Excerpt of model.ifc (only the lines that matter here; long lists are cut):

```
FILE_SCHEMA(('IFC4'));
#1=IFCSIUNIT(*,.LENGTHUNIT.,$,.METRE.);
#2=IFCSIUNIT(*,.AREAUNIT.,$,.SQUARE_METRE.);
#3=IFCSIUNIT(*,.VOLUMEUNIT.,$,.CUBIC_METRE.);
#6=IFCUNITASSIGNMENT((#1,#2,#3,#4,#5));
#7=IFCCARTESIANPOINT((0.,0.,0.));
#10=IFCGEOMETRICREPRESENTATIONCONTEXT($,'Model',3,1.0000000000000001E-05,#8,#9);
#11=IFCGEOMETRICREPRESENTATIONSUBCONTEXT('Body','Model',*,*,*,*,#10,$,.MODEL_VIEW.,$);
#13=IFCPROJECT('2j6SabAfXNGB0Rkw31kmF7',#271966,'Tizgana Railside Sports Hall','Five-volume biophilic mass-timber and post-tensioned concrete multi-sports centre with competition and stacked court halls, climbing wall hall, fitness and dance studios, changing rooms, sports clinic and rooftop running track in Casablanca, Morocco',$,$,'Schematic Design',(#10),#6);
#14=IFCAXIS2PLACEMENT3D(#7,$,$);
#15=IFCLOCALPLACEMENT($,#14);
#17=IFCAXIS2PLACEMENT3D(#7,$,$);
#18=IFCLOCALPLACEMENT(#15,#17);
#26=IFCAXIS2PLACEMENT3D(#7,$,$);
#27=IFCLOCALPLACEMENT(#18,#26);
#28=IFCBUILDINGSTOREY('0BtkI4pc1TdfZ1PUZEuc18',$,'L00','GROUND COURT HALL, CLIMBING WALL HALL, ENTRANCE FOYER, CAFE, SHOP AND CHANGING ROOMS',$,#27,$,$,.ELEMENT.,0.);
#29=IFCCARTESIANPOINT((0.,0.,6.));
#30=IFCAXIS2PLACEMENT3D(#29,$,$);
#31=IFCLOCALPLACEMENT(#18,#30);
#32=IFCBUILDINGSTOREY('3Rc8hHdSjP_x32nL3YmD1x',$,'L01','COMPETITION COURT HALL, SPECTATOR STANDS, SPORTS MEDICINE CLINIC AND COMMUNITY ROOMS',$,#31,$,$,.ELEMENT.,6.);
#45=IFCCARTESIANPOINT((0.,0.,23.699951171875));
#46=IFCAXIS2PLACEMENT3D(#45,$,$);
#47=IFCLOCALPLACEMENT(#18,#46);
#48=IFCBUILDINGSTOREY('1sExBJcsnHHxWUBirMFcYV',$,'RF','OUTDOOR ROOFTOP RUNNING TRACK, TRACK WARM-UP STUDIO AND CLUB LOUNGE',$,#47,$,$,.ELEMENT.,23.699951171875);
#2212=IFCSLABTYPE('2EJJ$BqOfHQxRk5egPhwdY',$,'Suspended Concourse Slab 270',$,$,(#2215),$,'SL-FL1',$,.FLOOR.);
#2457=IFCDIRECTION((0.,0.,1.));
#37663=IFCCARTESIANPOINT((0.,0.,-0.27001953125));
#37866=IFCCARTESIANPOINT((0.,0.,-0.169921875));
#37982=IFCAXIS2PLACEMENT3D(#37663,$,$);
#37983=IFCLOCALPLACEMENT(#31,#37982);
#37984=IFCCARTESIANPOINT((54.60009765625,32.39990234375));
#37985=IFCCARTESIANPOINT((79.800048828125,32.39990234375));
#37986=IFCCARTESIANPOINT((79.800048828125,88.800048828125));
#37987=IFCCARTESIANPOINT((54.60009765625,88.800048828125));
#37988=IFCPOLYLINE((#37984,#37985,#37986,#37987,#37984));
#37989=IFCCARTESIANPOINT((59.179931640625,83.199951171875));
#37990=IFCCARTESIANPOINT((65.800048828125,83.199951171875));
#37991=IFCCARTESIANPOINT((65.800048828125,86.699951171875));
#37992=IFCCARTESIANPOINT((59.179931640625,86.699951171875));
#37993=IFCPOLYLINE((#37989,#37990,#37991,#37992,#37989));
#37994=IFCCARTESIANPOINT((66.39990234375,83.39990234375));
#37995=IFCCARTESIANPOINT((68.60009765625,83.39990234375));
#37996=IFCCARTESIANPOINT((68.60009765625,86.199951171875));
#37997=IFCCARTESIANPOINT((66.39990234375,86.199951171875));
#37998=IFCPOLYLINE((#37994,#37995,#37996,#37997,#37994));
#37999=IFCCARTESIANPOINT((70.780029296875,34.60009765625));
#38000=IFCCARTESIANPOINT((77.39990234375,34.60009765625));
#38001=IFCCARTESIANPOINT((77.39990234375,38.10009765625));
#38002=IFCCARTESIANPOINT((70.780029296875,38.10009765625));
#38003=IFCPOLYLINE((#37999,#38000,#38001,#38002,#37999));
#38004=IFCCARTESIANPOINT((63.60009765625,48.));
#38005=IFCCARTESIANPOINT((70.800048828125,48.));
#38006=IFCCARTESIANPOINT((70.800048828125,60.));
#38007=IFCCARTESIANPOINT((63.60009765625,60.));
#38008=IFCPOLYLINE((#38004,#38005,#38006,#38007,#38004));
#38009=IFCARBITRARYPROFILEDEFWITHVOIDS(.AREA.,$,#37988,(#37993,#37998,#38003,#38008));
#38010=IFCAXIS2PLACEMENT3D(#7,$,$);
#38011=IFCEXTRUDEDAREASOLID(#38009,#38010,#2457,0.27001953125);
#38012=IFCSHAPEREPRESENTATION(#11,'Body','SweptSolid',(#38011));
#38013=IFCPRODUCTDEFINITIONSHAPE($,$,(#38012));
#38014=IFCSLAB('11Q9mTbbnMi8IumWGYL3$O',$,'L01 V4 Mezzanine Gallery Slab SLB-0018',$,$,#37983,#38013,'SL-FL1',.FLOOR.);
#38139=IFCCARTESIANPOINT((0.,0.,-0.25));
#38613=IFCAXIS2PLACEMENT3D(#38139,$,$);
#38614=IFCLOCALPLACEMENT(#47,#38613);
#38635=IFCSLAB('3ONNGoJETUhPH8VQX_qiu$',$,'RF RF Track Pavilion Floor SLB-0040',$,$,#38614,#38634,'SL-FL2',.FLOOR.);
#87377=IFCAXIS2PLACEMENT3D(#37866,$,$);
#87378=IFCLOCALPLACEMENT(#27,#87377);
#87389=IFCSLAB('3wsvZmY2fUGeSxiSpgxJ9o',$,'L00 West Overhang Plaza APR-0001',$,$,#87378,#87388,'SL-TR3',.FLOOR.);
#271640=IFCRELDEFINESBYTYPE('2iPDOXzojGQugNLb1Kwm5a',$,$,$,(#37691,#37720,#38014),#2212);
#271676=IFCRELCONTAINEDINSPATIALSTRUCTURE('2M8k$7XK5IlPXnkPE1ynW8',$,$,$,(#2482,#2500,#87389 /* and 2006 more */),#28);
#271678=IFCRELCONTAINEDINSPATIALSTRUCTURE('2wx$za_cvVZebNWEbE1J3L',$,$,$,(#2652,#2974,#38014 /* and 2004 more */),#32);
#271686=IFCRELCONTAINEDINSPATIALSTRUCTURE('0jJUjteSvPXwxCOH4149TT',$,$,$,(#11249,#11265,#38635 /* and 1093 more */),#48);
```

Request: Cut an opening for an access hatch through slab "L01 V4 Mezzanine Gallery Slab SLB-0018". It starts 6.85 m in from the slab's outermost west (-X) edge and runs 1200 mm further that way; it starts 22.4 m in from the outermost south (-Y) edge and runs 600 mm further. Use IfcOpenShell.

```python
import numpy as np
import ifcopenshell
import ifcopenshell.api.feature
import ifcopenshell.api.geometry
import ifcopenshell.api.root
import ifcopenshell.geom
import ifcopenshell.util.placement
import ifcopenshell.util.representation
import ifcopenshell.util.shape
import ifcopenshell.util.unit

model = ifcopenshell.open("model.ifc")
unit_scale = ifcopenshell.util.unit.calculate_unit_scale(model)
settings = ifcopenshell.geom.settings()


def volume(element):
    """Net volume in cubic metres, openings subtracted."""
    shape = ifcopenshell.geom.create_shape(settings, element)
    return ifcopenshell.util.shape.get_volume(shape.geometry)


slab = model.by_id(38014)
before = volume(slab)

# Extent in the slab's own axes, in metres. The edges named are its -X and -Y sides.
slab_shape = ifcopenshell.geom.create_shape(settings, slab)
vertices = ifcopenshell.util.shape.get_vertices(slab_shape.geometry)
x_min, y_min, bottom = vertices.min(axis=0)
top = vertices[:, 2].max()

opening = ifcopenshell.api.root.create_entity(model, ifc_class="IfcOpeningElement", name="Access hatch opening", predefined_type="OPENING")
context = ifcopenshell.util.representation.get_context(model, "Model", "Body", "MODEL_VIEW")
width, depth = 1.2, 0.6
outline = [(0.0, 0.0), (width, 0.0), (width, depth), (0.0, depth), (0.0, 0.0)]
# Overshoot both faces by 50 mm so the cut is clean.
shape = ifcopenshell.api.geometry.add_slab_representation(
    model, context=context, depth=top - bottom + 0.1, polyline=outline
)
ifcopenshell.api.geometry.assign_representation(model, product=opening, representation=shape)

matrix = ifcopenshell.util.placement.get_local_placement(slab.ObjectPlacement)
matrix[:, 3] = matrix @ np.append(np.array([x_min + 6.85, y_min + 22.4, bottom - 0.05]) / unit_scale, 1.0)
ifcopenshell.api.geometry.edit_object_placement(model, product=opening, matrix=matrix, is_si=False)
ifcopenshell.api.feature.add_feature(model, feature=opening, element=slab)

after = volume(slab)

print(f"slab volume {before:.3f} -> {after:.3f} m3")

model.write("model_updated.ifc")
```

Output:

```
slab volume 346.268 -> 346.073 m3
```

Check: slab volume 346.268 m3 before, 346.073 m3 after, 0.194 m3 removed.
